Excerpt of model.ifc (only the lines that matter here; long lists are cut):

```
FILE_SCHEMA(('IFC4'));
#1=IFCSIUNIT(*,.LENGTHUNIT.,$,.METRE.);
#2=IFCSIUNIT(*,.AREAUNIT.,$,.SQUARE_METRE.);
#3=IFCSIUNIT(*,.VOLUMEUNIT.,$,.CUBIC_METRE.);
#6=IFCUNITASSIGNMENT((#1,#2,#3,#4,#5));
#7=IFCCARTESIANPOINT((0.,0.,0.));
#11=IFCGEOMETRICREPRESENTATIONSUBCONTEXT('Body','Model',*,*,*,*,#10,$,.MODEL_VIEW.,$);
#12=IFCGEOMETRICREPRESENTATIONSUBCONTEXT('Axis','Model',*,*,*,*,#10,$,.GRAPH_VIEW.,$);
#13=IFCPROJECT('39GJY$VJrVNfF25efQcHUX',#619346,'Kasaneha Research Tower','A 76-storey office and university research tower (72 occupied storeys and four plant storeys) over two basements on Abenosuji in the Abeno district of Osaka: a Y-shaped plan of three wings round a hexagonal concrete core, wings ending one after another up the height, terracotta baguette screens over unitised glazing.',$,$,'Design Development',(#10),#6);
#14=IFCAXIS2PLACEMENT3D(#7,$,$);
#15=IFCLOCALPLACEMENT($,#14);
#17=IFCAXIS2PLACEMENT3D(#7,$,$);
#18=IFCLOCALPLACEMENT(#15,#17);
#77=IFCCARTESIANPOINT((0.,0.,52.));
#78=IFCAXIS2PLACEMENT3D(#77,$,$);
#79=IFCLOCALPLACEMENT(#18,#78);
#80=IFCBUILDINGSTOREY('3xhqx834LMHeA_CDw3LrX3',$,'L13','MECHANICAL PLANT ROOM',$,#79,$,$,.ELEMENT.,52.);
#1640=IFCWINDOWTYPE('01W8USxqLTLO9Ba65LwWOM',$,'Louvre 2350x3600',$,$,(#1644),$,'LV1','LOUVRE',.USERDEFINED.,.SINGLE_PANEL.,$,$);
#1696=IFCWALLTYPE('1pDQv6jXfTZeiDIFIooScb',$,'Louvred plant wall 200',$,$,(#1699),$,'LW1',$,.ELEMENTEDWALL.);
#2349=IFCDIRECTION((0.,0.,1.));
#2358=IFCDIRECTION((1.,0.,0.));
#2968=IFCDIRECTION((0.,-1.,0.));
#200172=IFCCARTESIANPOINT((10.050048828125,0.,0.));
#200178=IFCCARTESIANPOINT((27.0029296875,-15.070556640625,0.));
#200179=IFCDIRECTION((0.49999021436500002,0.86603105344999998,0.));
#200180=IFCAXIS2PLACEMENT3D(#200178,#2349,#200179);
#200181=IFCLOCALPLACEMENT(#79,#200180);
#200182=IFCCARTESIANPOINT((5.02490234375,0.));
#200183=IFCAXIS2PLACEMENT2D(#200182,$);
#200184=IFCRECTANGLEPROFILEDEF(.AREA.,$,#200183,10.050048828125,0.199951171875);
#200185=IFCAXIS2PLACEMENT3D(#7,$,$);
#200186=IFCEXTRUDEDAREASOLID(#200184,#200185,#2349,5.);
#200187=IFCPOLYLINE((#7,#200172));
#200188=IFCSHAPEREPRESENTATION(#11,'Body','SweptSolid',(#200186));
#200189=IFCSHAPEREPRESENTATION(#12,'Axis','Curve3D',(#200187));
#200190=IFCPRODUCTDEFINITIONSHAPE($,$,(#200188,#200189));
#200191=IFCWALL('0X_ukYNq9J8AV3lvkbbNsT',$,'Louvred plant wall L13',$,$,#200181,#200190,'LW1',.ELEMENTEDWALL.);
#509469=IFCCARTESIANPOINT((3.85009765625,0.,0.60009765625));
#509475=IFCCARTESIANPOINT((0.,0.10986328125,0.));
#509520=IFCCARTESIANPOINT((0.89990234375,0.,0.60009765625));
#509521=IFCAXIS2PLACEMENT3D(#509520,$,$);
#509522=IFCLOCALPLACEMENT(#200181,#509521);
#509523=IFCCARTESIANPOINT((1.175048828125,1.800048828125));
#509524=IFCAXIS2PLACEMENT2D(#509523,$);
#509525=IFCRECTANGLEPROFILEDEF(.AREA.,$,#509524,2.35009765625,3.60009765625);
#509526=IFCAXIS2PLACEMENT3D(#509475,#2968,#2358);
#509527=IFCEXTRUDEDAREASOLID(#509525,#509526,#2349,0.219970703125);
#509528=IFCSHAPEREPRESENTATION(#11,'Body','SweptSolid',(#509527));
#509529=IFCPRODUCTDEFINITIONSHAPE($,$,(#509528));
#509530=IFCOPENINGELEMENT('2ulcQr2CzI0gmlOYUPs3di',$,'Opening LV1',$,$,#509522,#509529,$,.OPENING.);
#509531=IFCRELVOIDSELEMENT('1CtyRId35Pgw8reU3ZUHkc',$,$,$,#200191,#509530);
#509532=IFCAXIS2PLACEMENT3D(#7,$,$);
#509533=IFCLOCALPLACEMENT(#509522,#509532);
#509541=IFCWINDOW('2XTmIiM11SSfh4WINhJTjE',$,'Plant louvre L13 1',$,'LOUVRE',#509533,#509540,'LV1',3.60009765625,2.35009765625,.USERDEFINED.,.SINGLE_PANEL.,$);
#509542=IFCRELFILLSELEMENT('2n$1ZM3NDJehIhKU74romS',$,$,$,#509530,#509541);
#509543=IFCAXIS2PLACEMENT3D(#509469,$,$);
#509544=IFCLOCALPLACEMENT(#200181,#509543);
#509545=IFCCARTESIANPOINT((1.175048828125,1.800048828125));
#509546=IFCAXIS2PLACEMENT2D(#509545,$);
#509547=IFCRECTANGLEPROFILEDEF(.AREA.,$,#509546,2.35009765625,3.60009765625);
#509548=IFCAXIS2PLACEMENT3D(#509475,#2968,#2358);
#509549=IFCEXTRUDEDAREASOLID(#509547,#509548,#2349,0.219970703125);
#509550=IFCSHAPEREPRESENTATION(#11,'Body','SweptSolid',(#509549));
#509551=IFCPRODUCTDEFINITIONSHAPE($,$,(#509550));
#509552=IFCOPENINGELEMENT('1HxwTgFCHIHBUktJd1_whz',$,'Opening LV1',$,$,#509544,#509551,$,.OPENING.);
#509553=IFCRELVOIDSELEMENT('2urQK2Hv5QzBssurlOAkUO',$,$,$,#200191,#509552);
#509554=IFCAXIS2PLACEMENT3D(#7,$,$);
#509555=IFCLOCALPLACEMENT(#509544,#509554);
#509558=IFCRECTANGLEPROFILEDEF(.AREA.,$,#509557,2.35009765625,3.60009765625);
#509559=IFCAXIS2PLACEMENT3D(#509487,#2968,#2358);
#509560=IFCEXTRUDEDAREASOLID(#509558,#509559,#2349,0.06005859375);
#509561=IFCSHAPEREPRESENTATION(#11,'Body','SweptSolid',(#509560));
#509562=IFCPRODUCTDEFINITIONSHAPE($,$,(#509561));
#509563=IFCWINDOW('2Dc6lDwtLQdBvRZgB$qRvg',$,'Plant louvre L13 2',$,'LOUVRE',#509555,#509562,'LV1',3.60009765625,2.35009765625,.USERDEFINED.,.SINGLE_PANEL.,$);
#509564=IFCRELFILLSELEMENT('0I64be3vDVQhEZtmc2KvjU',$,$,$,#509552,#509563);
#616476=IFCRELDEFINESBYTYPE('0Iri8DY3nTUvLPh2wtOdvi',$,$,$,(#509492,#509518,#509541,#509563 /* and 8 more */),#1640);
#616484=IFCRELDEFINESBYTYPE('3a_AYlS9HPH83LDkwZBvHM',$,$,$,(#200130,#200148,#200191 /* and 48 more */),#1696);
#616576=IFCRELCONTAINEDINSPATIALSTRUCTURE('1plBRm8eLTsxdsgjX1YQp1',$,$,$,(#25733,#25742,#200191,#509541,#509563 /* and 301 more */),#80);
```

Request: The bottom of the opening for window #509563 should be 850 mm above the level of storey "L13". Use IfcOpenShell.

```python
import numpy as np
import ifcopenshell
import ifcopenshell.api.geometry
import ifcopenshell.geom
import ifcopenshell.util.element
import ifcopenshell.util.placement
import ifcopenshell.util.shape
import ifcopenshell.util.unit

model = ifcopenshell.open("model.ifc")
unit_scale = ifcopenshell.util.unit.calculate_unit_scale(model)

window = model.by_guid("2Dc6lDwtLQdBvRZgB$qRvg")
opening = window.FillsVoids[0].RelatingOpeningElement
storey = ifcopenshell.util.element.get_container(window, ifc_class="IfcBuildingStorey")
level = ifcopenshell.util.placement.get_local_placement(storey.ObjectPlacement)[2, 3]

# The opening's origin need not be at the sill, so measure its lowest point.
shape = ifcopenshell.geom.create_shape(ifcopenshell.geom.settings(), opening)
bottom = ifcopenshell.util.shape.get_shape_bottom_elevation(shape, shape.geometry) / unit_scale
dz = level + 0.85 - bottom

shift = np.array([0.0, 0.0, dz])
# The window is placed relative to its opening, so it follows when the opening moves.
matrix = ifcopenshell.util.placement.get_local_placement(opening.ObjectPlacement)
matrix[:3, 3] += shift
ifcopenshell.api.geometry.edit_object_placement(
    model, product=opening, matrix=matrix, is_si=False, should_transform_children=True
)

print(f"moved by {dz * unit_scale:+.3f} m")

model.write("model_edited.ifc")
```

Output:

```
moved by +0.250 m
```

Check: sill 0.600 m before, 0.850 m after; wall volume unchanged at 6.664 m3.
